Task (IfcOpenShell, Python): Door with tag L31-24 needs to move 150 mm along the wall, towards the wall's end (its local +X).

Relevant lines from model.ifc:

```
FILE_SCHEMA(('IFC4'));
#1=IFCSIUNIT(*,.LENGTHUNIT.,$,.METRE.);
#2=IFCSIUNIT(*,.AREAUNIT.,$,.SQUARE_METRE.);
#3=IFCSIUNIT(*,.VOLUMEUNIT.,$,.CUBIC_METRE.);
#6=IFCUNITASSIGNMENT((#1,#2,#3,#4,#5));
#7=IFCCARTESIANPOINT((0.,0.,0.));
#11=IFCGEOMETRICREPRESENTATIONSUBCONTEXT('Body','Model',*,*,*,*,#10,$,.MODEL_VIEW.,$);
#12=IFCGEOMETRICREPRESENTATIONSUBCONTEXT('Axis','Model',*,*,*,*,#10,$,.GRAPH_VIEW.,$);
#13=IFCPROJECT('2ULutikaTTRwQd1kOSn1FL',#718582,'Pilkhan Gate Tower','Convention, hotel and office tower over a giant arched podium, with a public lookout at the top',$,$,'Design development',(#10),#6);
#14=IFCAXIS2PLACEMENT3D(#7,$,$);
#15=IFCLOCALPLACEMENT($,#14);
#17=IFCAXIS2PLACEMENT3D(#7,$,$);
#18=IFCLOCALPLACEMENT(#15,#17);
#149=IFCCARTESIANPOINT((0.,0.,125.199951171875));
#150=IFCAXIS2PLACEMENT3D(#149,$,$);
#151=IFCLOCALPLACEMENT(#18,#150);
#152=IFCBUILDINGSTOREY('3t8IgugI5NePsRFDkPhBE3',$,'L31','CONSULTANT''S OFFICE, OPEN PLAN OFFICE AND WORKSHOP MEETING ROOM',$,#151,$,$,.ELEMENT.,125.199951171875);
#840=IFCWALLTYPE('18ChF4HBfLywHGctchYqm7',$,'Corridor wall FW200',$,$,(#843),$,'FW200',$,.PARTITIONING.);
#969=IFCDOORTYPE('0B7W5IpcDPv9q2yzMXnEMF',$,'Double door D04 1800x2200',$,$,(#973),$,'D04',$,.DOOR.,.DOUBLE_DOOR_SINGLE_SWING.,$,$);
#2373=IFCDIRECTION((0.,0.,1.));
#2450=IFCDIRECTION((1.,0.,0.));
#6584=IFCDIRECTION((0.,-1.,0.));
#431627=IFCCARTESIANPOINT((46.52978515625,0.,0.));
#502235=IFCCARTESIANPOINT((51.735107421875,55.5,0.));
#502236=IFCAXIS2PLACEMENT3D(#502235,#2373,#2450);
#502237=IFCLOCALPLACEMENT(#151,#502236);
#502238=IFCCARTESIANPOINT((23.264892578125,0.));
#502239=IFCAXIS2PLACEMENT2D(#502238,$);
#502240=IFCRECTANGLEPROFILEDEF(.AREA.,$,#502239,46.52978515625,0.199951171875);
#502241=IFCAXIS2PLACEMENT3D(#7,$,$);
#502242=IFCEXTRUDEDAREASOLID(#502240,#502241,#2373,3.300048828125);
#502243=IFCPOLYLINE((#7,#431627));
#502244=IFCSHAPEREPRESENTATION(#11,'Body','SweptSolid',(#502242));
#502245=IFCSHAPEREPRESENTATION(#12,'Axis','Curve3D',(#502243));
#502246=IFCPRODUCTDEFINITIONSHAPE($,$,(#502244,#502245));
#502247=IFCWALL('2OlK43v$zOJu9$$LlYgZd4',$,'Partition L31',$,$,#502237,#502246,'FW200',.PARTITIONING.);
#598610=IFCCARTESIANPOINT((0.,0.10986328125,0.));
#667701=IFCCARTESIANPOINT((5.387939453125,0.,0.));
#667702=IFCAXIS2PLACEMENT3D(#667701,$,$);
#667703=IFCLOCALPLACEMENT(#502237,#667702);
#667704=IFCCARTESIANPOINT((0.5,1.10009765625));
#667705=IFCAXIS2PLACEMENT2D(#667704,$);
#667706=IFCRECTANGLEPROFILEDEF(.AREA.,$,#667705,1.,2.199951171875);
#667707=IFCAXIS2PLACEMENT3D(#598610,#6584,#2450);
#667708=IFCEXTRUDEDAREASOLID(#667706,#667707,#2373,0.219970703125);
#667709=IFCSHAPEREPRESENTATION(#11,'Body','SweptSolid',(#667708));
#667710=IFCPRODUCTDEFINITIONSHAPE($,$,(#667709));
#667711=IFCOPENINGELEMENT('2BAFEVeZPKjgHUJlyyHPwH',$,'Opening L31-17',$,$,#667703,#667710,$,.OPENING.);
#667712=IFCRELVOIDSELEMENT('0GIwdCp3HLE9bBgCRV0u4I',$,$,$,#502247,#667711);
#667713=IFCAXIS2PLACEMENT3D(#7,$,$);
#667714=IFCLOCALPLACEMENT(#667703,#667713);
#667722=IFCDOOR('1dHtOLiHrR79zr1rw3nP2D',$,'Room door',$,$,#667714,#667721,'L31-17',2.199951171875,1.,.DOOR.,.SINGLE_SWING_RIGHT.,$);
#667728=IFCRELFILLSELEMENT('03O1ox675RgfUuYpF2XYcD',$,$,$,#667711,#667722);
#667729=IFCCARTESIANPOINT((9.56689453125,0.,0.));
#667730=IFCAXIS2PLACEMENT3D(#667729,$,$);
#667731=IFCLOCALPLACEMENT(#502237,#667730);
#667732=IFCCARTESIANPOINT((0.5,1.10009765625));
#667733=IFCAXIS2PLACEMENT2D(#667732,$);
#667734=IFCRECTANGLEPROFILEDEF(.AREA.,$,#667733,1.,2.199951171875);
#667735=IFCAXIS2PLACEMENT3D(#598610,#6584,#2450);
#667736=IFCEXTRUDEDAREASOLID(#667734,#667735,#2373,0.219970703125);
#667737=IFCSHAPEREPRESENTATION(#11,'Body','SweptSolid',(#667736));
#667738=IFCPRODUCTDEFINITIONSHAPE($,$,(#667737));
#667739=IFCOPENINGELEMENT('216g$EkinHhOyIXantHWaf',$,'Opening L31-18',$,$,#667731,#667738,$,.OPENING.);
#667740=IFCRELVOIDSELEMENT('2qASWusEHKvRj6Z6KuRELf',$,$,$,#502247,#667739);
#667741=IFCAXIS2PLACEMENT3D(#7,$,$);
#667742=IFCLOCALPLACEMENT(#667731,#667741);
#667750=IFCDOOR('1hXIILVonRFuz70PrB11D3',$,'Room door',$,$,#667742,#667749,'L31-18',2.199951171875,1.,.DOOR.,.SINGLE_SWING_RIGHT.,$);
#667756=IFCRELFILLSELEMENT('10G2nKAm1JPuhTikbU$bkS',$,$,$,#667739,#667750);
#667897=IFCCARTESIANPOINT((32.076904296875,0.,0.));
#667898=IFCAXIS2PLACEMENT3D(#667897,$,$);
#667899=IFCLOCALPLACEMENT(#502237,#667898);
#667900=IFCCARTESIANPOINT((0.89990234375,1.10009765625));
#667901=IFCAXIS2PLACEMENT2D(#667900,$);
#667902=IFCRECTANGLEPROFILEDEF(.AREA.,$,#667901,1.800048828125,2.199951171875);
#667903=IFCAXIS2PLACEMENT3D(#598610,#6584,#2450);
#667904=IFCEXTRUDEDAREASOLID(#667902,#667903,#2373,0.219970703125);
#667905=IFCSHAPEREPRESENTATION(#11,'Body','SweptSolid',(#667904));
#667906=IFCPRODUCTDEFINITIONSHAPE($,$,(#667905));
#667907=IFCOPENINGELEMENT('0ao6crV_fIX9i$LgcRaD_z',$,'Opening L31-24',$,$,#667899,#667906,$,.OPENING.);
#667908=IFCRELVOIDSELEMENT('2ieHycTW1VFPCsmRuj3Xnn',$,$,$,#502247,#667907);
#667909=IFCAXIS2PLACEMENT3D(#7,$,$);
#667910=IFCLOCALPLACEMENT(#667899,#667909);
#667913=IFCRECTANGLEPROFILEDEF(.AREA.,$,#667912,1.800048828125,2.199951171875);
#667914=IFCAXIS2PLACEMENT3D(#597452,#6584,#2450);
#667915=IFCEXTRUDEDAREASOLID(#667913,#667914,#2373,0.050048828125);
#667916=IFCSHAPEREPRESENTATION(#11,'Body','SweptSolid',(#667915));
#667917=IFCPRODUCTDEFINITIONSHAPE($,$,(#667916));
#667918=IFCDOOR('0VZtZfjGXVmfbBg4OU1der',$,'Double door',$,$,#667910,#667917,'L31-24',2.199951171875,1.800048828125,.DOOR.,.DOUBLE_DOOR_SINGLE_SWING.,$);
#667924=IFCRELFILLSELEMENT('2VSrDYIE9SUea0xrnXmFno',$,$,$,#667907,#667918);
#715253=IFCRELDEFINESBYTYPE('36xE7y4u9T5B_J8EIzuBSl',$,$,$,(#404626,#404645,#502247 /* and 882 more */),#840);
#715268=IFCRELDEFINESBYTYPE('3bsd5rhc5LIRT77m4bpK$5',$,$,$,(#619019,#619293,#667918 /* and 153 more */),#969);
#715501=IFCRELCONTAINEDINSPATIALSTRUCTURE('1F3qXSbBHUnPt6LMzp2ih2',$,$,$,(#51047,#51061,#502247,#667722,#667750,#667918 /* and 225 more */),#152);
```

```python
import ifcopenshell
import ifcopenshell.api.geometry
import ifcopenshell.util.placement
import ifcopenshell.util.unit

model = ifcopenshell.open("model.ifc")
unit_scale = ifcopenshell.util.unit.calculate_unit_scale(model)

door = model.by_guid("0VZtZfjGXVmfbBg4OU1der")
opening = door.FillsVoids[0].RelatingOpeningElement
wall = opening.VoidsElements[0].RelatingBuildingElement

wall_matrix = ifcopenshell.util.placement.get_local_placement(wall.ObjectPlacement)
shift = wall_matrix[:3, 0] * 0.15 / unit_scale
before = ifcopenshell.util.placement.get_local_placement(door.ObjectPlacement)[:3, 3].copy()

# The door is placed relative to its opening, so it follows when the opening moves.
matrix = ifcopenshell.util.placement.get_local_placement(opening.ObjectPlacement)
matrix[:3, 3] += shift
ifcopenshell.api.geometry.edit_object_placement(
    model, product=opening, matrix=matrix, is_si=False, should_transform_children=True
)

after = ifcopenshell.util.placement.get_local_placement(door.ObjectPlacement)[:3, 3]
print("door moved by", (after - before).round(3) + 0.0)

model.write("model_rev.ifc")
```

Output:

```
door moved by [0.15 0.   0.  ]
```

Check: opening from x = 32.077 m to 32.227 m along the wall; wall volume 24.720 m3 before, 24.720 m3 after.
